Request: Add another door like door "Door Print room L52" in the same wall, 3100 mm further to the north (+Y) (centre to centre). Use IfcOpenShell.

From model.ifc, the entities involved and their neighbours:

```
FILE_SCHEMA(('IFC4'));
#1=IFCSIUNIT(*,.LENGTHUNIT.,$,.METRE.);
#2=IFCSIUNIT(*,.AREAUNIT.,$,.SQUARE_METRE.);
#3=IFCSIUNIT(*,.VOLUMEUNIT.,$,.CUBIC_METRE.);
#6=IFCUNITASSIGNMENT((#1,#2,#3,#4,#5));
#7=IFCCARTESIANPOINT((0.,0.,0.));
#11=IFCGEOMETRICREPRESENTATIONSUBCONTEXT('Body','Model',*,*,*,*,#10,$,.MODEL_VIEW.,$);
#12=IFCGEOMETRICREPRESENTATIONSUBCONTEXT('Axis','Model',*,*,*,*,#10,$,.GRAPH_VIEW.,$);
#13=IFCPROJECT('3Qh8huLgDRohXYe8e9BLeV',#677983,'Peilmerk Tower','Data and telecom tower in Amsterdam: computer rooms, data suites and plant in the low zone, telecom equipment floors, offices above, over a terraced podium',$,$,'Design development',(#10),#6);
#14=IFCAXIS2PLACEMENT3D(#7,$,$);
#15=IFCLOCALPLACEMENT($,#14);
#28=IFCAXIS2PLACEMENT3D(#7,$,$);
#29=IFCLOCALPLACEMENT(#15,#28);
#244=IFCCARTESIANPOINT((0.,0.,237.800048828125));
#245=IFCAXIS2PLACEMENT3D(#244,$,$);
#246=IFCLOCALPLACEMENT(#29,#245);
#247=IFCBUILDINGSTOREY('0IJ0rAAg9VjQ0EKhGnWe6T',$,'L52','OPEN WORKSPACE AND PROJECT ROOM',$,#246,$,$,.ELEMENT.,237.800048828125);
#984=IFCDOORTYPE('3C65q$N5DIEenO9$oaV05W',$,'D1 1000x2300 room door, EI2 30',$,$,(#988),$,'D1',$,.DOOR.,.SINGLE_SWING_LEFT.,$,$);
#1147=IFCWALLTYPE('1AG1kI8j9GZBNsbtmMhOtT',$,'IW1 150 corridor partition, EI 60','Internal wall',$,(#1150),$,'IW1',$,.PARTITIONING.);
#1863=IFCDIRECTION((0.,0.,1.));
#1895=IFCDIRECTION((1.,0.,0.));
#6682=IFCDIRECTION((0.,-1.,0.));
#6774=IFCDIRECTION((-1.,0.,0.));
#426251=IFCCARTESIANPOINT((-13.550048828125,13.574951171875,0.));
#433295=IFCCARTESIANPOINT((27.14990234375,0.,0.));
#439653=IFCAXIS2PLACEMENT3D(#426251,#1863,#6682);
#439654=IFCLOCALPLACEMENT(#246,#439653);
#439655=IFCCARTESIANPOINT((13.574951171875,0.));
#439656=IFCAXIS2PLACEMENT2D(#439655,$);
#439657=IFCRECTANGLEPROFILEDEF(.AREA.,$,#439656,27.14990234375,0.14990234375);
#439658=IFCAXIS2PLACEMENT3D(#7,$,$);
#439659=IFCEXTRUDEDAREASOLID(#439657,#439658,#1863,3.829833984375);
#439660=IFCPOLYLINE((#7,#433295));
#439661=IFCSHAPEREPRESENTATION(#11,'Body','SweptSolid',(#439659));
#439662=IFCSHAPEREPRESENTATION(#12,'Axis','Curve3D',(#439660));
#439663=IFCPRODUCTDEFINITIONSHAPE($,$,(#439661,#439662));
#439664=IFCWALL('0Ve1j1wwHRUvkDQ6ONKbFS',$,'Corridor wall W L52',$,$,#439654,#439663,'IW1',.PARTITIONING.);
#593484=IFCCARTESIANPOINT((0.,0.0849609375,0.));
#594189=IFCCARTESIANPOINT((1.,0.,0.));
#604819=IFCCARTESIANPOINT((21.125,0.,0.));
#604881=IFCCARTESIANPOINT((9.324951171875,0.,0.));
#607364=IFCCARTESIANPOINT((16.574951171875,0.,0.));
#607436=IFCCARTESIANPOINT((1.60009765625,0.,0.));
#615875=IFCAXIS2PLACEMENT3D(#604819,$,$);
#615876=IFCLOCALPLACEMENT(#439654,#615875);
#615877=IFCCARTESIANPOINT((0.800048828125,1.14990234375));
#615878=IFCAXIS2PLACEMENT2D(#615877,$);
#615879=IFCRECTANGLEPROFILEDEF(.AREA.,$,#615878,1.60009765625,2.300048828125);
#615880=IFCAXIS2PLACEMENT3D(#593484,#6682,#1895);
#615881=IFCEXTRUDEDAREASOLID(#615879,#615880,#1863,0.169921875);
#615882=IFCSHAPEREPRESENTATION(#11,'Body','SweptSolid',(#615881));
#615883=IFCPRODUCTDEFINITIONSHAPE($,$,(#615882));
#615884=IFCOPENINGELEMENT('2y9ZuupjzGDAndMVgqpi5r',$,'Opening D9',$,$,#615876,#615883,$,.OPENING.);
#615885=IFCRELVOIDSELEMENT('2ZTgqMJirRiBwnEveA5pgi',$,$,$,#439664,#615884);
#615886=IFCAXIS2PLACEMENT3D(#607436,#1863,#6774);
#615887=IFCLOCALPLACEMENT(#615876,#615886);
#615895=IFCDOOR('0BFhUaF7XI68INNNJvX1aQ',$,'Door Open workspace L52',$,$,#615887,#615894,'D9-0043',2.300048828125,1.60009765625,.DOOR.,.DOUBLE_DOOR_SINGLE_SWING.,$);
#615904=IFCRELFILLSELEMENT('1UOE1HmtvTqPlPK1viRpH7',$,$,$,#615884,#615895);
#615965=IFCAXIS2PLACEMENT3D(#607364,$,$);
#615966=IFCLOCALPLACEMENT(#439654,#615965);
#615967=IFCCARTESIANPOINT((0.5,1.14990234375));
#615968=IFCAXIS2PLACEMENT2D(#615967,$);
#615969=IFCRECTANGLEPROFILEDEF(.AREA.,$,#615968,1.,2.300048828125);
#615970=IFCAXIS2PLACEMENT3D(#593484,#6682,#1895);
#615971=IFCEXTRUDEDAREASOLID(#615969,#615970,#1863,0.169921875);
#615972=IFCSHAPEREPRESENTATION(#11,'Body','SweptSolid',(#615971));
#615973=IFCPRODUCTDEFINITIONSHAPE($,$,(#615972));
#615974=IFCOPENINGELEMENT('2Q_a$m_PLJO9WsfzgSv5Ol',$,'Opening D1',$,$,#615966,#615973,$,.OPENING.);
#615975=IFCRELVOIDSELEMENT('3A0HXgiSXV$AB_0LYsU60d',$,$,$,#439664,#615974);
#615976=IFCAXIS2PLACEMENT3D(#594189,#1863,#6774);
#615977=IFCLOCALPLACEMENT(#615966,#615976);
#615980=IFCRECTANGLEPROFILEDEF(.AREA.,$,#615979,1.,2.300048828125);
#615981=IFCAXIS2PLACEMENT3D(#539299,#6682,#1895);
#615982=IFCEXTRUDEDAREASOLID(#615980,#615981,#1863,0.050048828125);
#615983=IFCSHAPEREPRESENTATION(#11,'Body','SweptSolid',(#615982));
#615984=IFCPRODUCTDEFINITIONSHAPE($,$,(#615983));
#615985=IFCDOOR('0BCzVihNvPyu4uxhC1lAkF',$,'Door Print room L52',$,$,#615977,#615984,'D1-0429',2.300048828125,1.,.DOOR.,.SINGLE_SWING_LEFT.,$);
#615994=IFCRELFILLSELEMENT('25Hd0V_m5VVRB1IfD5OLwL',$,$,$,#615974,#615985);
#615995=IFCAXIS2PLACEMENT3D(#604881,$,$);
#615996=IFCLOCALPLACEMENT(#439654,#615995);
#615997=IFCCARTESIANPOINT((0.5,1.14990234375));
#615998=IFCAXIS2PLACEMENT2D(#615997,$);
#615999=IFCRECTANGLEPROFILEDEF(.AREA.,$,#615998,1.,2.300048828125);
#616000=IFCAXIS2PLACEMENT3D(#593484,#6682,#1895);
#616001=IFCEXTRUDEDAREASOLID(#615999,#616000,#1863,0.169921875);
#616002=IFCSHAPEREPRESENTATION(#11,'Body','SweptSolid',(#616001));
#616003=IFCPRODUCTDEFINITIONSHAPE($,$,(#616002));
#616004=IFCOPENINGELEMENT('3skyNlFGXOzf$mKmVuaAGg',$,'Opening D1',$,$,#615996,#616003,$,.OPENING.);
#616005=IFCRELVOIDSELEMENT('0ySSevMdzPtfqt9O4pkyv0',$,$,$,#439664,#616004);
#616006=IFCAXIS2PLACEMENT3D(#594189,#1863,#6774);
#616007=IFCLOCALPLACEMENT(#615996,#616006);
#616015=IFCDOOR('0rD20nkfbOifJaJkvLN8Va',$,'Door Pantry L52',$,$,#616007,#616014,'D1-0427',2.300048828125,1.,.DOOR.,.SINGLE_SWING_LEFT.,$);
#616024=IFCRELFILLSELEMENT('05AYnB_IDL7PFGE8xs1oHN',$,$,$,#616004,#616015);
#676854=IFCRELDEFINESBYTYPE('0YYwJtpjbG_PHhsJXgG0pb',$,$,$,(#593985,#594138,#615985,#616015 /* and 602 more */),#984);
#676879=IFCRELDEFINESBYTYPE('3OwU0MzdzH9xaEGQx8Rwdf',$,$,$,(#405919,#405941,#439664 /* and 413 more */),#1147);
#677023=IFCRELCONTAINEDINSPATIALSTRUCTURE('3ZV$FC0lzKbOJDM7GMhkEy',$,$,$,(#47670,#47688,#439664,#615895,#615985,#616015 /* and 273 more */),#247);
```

```python
import ifcopenshell
import ifcopenshell.api.feature
import ifcopenshell.api.geometry
import ifcopenshell.api.root
import ifcopenshell.geom
import ifcopenshell.util.element
import ifcopenshell.util.placement
import ifcopenshell.util.shape
import ifcopenshell.util.unit

model = ifcopenshell.open("model.ifc")
unit_scale = ifcopenshell.util.unit.calculate_unit_scale(model)
settings = ifcopenshell.geom.settings()


def volume(element):
    """Net volume in cubic metres, openings subtracted."""
    shape = ifcopenshell.geom.create_shape(settings, element)
    return ifcopenshell.util.shape.get_volume(shape.geometry)


door = model.by_guid("0BCzVihNvPyu4uxhC1lAkF")
opening = door.FillsVoids[0].RelatingOpeningElement
wall = opening.VoidsElements[0].RelatingBuildingElement
before = volume(wall)
shift = ifcopenshell.util.placement.get_local_placement(wall.ObjectPlacement)[:3, 0] * -3.1 / unit_scale

# copy_class copies the void relationship, type, container and properties, but no geometry.
new_opening = ifcopenshell.api.root.copy_class(model, product=opening)
new_opening.Representation = ifcopenshell.util.element.copy_deep(
    model, opening.Representation, exclude=["IfcGeometricRepresentationContext", "IfcRepresentationMap"]
)
new_door = ifcopenshell.api.root.copy_class(model, product=door)
new_door.Representation = ifcopenshell.util.element.copy_deep(
    model, door.Representation, exclude=["IfcGeometricRepresentationContext", "IfcRepresentationMap"]
)
new_door.Tag = None
ifcopenshell.api.feature.add_filling(model, opening=new_opening, element=new_door)

for old, new in ((opening, new_opening), (door, new_door)):
    matrix = ifcopenshell.util.placement.get_local_placement(old.ObjectPlacement)
    matrix[:3, 3] += shift
    ifcopenshell.api.geometry.edit_object_placement(model, product=new, matrix=matrix, is_si=False)

after = volume(wall)

print(f"wall volume {before:.3f} -> {after:.3f} m3")

model.write("model_v2.ifc")
```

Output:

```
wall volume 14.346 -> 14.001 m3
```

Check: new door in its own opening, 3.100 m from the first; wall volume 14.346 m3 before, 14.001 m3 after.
